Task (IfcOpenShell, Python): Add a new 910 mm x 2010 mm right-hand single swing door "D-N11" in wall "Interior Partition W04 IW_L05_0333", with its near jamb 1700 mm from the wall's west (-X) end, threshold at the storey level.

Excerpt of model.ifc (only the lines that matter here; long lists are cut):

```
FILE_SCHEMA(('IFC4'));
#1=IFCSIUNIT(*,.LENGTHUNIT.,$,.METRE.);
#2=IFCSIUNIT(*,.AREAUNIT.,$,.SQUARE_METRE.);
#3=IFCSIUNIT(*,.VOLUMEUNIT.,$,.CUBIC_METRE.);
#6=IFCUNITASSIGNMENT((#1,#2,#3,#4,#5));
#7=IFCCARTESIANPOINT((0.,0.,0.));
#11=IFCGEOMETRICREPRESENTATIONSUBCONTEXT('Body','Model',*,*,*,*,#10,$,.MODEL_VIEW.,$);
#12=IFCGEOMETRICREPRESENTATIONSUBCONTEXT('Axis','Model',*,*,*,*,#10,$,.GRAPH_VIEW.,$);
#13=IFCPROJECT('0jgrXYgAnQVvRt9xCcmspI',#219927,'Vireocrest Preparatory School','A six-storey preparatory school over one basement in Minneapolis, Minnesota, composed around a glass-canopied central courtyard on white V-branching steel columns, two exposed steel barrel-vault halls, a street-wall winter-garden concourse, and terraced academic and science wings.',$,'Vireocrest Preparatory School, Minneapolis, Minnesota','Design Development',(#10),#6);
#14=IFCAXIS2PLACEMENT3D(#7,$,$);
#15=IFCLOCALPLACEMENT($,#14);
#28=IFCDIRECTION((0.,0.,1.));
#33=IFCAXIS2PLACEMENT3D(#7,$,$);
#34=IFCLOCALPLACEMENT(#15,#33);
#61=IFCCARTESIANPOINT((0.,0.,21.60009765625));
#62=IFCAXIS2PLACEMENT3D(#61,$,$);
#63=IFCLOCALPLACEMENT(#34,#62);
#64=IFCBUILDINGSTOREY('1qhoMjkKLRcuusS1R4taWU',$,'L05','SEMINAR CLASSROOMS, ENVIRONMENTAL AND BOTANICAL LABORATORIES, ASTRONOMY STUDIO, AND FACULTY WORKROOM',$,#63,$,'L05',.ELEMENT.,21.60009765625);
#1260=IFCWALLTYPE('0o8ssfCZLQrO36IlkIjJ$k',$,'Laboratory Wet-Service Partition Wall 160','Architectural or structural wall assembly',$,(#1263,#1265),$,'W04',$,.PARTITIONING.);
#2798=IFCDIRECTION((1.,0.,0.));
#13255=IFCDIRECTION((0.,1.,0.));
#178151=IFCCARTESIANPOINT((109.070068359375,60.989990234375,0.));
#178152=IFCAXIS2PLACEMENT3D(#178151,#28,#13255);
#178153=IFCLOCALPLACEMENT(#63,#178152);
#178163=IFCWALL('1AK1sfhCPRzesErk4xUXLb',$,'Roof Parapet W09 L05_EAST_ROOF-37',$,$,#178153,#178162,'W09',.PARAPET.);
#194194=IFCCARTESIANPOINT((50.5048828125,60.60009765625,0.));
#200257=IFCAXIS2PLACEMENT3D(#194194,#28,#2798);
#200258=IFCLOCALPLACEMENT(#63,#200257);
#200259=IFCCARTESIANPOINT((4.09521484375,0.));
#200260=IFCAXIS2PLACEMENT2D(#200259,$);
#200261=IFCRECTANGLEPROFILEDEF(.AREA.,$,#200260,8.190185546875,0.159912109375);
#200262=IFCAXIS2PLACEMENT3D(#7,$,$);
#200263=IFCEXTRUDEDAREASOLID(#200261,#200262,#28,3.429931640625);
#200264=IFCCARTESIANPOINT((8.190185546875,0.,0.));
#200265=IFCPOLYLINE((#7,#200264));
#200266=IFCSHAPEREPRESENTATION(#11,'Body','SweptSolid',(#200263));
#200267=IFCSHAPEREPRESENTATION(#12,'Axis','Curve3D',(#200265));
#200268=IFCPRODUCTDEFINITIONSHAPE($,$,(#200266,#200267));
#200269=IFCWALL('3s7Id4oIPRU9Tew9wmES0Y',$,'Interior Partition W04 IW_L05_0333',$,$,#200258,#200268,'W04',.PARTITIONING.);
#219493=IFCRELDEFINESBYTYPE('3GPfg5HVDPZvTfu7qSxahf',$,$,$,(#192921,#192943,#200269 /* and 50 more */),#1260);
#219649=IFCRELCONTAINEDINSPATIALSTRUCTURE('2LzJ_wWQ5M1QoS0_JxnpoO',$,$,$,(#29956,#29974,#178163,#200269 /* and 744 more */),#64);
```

```python
import numpy as np
import ifcopenshell
import ifcopenshell.api.feature
import ifcopenshell.api.geometry
import ifcopenshell.api.root
import ifcopenshell.api.spatial
import ifcopenshell.geom
import ifcopenshell.util.element
import ifcopenshell.util.placement
import ifcopenshell.util.representation
import ifcopenshell.util.shape
import ifcopenshell.util.unit

model = ifcopenshell.open("model.ifc")
unit_scale = ifcopenshell.util.unit.calculate_unit_scale(model)
settings = ifcopenshell.geom.settings()


def volume(element):
    """Net volume in cubic metres, openings subtracted."""
    shape = ifcopenshell.geom.create_shape(settings, element)
    return ifcopenshell.util.shape.get_volume(shape.geometry)


wall = model.by_guid("3s7Id4oIPRU9Tew9wmES0Y")
storey = ifcopenshell.util.element.get_container(wall, ifc_class="IfcBuildingStorey")
context = ifcopenshell.util.representation.get_context(model, "Model", "Body", "MODEL_VIEW")
before = volume(wall)

width, height, from_end, sill = 0.91, 2.01, 1.7, 0.0  # metres

# The wall runs along its own X axis, and the end named is its -X end.
wall_shape = ifcopenshell.geom.create_shape(settings, wall)
x, y, z = ifcopenshell.util.shape.get_vertices(wall_shape.geometry).T
start = x.min() + from_end
face, thickness = float(y.min()), float(y.max() - y.min())
wall_matrix = ifcopenshell.util.placement.get_local_placement(wall.ObjectPlacement)
level = ifcopenshell.util.placement.get_local_placement(storey.ObjectPlacement)[2, 3]


def in_wall(x, y):
    """Placement at x, y metres in the wall's axes, at sill height."""
    matrix = wall_matrix.copy()
    matrix[:, 3] = wall_matrix @ np.array([x / unit_scale, y / unit_scale, 0.0, 1.0])
    matrix[2, 3] = level + sill / unit_scale
    return matrix


# Opening: a box that overshoots both wall faces by 50 mm.
opening = ifcopenshell.api.root.create_entity(model, ifc_class="IfcOpeningElement", predefined_type="OPENING")
box = ifcopenshell.api.geometry.add_wall_representation(
    model, context=context, length=width, height=height, thickness=thickness + 0.1
)
ifcopenshell.api.geometry.assign_representation(model, product=opening, representation=box)
ifcopenshell.api.geometry.edit_object_placement(model, product=opening, matrix=in_wall(start, face - 0.05), is_si=False)
ifcopenshell.api.feature.add_feature(model, feature=opening, element=wall)

door = ifcopenshell.api.root.create_entity(model, ifc_class="IfcDoor", name="D-N11", predefined_type="DOOR")
door.OverallWidth, door.OverallHeight = width / unit_scale, height / unit_scale
door.OperationType = "SINGLE_SWING_RIGHT"
body = ifcopenshell.api.geometry.add_door_representation(
    model,
    context=context,
    overall_width=door.OverallWidth,
    overall_height=door.OverallHeight,
    operation_type="SINGLE_SWING_RIGHT",
    lining_properties={"LiningDepth": thickness / unit_scale, "ThresholdDepth": thickness / unit_scale},
)
ifcopenshell.api.geometry.assign_representation(model, product=door, representation=body)
ifcopenshell.api.spatial.assign_container(model, products=[door], relating_structure=storey)
ifcopenshell.api.feature.add_filling(model, opening=opening, element=door)

# The lining spans the wall, so the door starts at the wall face.
ifcopenshell.api.geometry.edit_object_placement(model, product=door, matrix=in_wall(start, face), is_si=False)

after = volume(wall)

print(f"wall volume {before:.3f} -> {after:.3f} m3")

model.write("model-out.ifc")
```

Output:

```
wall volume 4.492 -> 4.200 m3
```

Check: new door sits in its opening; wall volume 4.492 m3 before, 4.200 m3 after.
